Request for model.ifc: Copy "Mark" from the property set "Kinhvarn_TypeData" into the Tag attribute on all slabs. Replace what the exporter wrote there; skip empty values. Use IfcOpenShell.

First a look at what the model holds.

```python
import ifcopenshell
import ifcopenshell.util.element

model = ifcopenshell.open("model.ifc")
print(model.schema)
slabs = model.by_type("IfcSlab")
print(len(slabs), "slabs")
for e in slabs[:8]:
    source = ifcopenshell.util.element.get_pset(e, "Kinhvarn_TypeData", "Mark")
    target = e.Tag
    print(e.id(), repr(source), repr(target), sep=" | ")
```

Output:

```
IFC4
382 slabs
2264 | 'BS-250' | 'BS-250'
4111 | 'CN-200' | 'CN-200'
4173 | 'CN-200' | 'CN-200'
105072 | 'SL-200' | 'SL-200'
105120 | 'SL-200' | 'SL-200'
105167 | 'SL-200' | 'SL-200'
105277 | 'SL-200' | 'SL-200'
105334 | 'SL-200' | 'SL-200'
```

```python
import ifcopenshell
import ifcopenshell.util.element

model = ifcopenshell.open("model.ifc")

count = 0
for e in model.by_type("IfcSlab"):
    value = ifcopenshell.util.element.get_pset(e, "Kinhvarn_TypeData", "Mark")
    current = e.Tag
    if not value or not value.strip() or current == value:
        continue
    e.Tag = value
    count += 1

print(count, "slabs updated")

model.write("model-out.ifc")
```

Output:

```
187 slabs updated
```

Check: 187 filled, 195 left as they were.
